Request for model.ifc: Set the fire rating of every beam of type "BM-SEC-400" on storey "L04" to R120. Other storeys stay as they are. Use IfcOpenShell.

First a look at what the model holds.

```python
import ifcopenshell
import ifcopenshell.util.element

model = ifcopenshell.open("model.ifc")
print(model.schema)
storey = next(s for s in model.by_type("IfcBuildingStorey") if s.Name == "L04")
beams = [e for e in ifcopenshell.util.element.get_decomposition(storey) if e.is_a("IfcBeam")]
seen = {}
for e in beams:
    element_type = ifcopenshell.util.element.get_type(e)
    key = (element_type.Name if element_type != e and element_type else None, ifcopenshell.util.element.get_pset(e, "Pset_BeamCommon", "FireRating"))
    seen[key] = seen.get(key, 0) + 1
for (name, value), count in sorted(seen.items(), key=str):
    print(count, "x", name, "|", value)
```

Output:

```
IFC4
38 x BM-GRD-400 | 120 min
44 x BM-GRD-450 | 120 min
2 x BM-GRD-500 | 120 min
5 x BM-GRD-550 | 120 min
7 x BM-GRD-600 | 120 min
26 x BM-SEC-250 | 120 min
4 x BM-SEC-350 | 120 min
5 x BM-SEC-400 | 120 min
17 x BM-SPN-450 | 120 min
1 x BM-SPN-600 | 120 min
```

```python
import ifcopenshell
import ifcopenshell.api.pset
import ifcopenshell.util.element

model = ifcopenshell.open("model.ifc")

storey = next(s for s in model.by_type("IfcBuildingStorey") if s.Name == "L04")
beams = [e for e in ifcopenshell.util.element.get_decomposition(storey) if e.is_a("IfcBeam")]

count = 0
for e in beams:
    element_type = ifcopenshell.util.element.get_type(e)
    if element_type in (None, e) or element_type.Name != "BM-SEC-400":
        continue
    # add_pset returns the element's existing set when there is one.
    pset = ifcopenshell.api.pset.add_pset(model, product=e, name="Pset_BeamCommon")
    ifcopenshell.api.pset.edit_pset(model, pset=pset, properties={"FireRating": "R120"})
    count += 1

print(count, "beams updated")

model.write("model_rev.ifc")
```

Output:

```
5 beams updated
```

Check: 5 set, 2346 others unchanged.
